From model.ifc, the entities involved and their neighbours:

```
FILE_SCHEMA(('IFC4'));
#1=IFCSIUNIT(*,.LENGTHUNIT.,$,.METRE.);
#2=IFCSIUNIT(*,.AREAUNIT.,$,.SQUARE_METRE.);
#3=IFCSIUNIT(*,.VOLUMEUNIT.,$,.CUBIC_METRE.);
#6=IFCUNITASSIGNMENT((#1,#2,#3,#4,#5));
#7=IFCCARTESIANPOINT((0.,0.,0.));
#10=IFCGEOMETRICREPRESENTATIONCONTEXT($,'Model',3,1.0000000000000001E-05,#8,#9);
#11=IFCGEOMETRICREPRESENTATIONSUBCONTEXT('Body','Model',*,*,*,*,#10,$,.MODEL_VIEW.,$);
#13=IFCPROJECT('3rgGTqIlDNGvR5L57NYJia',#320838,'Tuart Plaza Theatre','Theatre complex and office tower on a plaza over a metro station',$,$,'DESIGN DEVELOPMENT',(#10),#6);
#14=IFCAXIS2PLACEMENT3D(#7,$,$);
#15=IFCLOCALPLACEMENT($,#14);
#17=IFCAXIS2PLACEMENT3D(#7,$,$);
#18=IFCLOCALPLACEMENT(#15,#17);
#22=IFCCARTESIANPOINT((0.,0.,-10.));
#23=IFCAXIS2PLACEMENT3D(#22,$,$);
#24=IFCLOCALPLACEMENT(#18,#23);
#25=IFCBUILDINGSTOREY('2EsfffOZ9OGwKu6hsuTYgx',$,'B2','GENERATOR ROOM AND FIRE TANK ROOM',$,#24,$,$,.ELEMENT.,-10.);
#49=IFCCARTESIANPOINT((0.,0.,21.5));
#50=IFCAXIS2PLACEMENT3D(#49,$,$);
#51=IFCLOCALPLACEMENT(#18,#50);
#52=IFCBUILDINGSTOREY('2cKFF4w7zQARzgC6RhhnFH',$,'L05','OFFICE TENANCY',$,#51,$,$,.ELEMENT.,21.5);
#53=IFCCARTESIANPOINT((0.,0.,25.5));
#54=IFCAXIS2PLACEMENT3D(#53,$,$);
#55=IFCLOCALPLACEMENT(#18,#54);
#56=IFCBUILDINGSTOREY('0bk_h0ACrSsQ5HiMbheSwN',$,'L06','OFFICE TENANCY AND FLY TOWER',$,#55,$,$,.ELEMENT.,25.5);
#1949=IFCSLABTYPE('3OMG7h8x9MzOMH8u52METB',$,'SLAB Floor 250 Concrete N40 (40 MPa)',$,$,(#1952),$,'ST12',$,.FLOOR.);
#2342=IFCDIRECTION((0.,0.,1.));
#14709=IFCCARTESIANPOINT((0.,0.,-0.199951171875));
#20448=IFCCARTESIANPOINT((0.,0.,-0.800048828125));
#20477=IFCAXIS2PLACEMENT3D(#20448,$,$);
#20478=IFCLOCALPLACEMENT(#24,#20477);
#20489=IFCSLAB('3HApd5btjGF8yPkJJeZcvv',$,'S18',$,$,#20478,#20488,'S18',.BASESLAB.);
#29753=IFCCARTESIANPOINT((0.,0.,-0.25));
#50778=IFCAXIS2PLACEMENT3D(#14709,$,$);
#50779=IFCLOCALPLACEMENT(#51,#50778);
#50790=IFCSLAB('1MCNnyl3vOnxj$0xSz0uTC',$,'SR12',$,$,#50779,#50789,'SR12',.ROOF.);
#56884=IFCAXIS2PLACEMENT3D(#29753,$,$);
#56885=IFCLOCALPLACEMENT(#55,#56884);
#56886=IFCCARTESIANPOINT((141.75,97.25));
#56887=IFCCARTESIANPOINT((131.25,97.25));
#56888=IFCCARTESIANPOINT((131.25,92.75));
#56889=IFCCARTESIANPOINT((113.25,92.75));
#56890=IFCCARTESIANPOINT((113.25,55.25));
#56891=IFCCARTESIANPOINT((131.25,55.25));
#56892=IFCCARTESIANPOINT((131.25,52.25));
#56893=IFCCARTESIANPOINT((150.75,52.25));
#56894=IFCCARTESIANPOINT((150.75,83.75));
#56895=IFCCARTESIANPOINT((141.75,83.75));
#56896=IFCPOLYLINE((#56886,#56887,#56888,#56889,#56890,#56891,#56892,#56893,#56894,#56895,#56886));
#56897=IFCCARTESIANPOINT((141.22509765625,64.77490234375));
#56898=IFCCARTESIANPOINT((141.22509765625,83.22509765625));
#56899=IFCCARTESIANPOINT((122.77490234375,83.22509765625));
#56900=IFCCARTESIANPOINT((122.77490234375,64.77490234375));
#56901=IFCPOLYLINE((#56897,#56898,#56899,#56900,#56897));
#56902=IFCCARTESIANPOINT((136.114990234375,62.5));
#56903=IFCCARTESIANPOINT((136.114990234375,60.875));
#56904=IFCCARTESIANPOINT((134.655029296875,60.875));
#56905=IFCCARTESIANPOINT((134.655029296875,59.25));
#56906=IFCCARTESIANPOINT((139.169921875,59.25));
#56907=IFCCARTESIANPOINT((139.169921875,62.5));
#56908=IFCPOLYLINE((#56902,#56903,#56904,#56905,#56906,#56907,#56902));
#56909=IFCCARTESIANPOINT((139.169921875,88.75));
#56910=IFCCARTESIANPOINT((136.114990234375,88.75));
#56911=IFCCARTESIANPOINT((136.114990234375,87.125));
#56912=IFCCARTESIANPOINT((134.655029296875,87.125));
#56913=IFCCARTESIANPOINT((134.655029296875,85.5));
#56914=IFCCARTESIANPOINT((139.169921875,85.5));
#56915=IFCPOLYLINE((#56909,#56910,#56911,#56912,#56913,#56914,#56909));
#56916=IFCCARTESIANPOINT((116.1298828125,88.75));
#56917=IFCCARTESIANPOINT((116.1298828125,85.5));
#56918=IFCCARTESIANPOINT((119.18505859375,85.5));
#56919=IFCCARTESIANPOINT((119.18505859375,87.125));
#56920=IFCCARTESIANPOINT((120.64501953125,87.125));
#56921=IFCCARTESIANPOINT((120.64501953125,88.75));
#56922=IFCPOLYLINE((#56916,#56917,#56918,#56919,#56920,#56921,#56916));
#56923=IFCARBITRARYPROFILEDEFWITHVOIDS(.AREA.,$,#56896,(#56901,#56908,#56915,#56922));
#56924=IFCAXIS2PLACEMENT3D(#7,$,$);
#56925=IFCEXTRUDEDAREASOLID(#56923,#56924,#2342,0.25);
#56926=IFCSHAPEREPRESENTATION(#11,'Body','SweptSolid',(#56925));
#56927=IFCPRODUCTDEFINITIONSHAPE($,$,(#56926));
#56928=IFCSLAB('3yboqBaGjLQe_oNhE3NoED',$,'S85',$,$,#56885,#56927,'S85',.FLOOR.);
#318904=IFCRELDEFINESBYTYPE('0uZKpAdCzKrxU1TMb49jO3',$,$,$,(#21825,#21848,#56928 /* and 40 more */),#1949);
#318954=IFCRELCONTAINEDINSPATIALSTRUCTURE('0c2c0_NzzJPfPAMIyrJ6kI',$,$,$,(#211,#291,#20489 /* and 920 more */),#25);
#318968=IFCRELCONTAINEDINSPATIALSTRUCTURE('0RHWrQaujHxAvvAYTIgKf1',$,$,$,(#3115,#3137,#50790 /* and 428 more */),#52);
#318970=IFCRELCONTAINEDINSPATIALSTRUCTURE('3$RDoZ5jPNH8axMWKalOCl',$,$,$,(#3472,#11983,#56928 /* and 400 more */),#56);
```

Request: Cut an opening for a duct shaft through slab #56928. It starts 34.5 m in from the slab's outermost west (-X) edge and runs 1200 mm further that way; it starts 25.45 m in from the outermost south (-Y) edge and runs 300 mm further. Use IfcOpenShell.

```python
import numpy as np
import ifcopenshell
import ifcopenshell.api.feature
import ifcopenshell.api.geometry
import ifcopenshell.api.root
import ifcopenshell.geom
import ifcopenshell.util.placement
import ifcopenshell.util.representation
import ifcopenshell.util.shape
import ifcopenshell.util.unit

model = ifcopenshell.open("model.ifc")
unit_scale = ifcopenshell.util.unit.calculate_unit_scale(model)
settings = ifcopenshell.geom.settings()


def volume(element):
    """Net volume in cubic metres, openings subtracted."""
    shape = ifcopenshell.geom.create_shape(settings, element)
    return ifcopenshell.util.shape.get_volume(shape.geometry)


slab = model.by_id(56928)
before = volume(slab)

# Extent in the slab's own axes, in metres. The edges named are its -X and -Y sides.
slab_shape = ifcopenshell.geom.create_shape(settings, slab)
vertices = ifcopenshell.util.shape.get_vertices(slab_shape.geometry)
x_min, y_min, bottom = vertices.min(axis=0)
top = vertices[:, 2].max()

opening = ifcopenshell.api.root.create_entity(model, ifc_class="IfcOpeningElement", name="Duct shaft opening", predefined_type="OPENING")
context = ifcopenshell.util.representation.get_context(model, "Model", "Body", "MODEL_VIEW")
width, depth = 1.2, 0.3
outline = [(0.0, 0.0), (width, 0.0), (width, depth), (0.0, depth), (0.0, 0.0)]
# Overshoot both faces by 50 mm so the cut is clean.
shape = ifcopenshell.api.geometry.add_slab_representation(
    model, context=context, depth=top - bottom + 0.1, polyline=outline
)
ifcopenshell.api.geometry.assign_representation(model, product=opening, representation=shape)

matrix = ifcopenshell.util.placement.get_local_placement(slab.ObjectPlacement)
matrix[:, 3] = matrix @ np.append(np.array([x_min + 34.5, y_min + 25.45, bottom - 0.05]) / unit_scale, 1.0)
ifcopenshell.api.geometry.edit_object_placement(model, product=opening, matrix=matrix, is_si=False)
ifcopenshell.api.feature.add_feature(model, feature=opening, element=slab)

after = volume(slab)

print(f"slab volume {before:.3f} -> {after:.3f} m3")

model.write("model_v2.ifc")
```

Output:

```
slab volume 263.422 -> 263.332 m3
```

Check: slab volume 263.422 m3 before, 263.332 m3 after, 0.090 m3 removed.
